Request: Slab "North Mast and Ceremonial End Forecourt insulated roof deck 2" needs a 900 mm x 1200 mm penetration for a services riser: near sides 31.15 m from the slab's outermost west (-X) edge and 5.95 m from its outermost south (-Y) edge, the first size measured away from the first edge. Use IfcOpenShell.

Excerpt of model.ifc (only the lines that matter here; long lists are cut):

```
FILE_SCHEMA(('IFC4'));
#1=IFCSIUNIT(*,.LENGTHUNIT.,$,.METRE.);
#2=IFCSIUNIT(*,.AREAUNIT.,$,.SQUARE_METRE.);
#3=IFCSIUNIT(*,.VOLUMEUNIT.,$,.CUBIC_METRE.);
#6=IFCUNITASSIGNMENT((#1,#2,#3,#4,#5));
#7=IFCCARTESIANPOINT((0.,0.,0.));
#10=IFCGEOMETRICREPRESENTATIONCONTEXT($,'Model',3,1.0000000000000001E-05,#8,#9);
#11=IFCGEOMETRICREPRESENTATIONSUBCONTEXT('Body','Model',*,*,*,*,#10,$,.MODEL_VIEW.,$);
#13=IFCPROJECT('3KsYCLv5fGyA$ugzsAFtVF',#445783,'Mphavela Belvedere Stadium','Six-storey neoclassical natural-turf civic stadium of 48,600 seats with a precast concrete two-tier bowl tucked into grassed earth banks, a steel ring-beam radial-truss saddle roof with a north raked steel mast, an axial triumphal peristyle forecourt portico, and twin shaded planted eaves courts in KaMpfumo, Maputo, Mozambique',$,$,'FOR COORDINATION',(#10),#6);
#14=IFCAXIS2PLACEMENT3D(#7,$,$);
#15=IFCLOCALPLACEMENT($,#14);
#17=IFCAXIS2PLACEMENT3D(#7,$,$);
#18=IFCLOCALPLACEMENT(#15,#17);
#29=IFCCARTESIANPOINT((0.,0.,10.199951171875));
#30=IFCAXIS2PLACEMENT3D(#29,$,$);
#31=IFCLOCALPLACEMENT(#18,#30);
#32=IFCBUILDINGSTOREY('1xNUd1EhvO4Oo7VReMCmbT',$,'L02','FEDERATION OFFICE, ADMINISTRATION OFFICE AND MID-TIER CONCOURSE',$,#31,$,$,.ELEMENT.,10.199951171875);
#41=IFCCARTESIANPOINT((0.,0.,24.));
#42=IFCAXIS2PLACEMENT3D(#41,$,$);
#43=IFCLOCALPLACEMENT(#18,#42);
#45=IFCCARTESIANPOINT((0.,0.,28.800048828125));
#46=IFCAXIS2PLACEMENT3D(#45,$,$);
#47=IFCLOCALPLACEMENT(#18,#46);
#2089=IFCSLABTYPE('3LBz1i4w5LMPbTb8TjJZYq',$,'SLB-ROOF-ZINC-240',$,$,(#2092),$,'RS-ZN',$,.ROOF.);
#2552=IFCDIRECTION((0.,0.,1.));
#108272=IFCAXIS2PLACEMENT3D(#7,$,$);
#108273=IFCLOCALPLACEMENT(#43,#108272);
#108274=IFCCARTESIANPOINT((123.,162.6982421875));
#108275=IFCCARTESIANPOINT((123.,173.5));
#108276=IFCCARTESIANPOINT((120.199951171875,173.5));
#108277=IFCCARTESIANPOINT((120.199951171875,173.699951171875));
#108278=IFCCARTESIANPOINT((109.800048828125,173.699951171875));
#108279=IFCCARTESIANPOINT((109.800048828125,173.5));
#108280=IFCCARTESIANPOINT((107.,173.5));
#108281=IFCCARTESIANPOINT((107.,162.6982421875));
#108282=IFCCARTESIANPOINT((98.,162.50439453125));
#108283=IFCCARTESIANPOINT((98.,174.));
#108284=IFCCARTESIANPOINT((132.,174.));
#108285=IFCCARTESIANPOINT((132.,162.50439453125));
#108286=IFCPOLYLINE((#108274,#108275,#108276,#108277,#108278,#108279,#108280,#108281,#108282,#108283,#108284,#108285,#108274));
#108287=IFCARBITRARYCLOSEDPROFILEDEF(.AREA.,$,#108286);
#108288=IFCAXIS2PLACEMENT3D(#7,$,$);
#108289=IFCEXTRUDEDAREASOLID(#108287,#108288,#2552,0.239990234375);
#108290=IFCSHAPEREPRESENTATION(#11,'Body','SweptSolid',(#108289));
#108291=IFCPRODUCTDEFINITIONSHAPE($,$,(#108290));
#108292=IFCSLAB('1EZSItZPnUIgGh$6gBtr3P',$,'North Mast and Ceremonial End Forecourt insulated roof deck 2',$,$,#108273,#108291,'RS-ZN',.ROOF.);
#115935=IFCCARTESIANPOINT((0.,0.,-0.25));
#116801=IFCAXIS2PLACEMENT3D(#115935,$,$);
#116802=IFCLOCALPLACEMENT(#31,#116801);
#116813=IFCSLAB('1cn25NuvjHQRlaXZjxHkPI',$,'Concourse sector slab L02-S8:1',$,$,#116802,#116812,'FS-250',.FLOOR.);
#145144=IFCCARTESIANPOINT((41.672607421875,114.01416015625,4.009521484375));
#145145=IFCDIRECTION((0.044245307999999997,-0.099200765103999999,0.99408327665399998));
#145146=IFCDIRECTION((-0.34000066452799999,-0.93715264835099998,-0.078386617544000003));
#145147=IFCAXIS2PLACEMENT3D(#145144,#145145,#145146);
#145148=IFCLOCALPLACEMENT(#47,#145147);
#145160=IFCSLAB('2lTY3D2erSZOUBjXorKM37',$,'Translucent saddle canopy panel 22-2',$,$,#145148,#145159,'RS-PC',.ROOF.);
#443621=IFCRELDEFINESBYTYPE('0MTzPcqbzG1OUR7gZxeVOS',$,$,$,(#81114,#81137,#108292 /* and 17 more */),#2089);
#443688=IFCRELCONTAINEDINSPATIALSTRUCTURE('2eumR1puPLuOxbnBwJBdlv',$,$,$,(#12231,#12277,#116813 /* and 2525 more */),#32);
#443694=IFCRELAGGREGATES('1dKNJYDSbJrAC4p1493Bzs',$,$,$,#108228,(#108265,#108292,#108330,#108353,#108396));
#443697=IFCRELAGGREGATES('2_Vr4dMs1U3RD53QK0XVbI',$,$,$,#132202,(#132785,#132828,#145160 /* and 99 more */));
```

```python
import numpy as np
import ifcopenshell
import ifcopenshell.api.feature
import ifcopenshell.api.geometry
import ifcopenshell.api.root
import ifcopenshell.geom
import ifcopenshell.util.placement
import ifcopenshell.util.representation
import ifcopenshell.util.shape
import ifcopenshell.util.unit

model = ifcopenshell.open("model.ifc")
unit_scale = ifcopenshell.util.unit.calculate_unit_scale(model)
settings = ifcopenshell.geom.settings()


def volume(element):
    """Net volume in cubic metres, openings subtracted."""
    shape = ifcopenshell.geom.create_shape(settings, element)
    return ifcopenshell.util.shape.get_volume(shape.geometry)


slab = model.by_guid("1EZSItZPnUIgGh$6gBtr3P")
before = volume(slab)

# Extent in the slab's own axes, in metres. The edges named are its -X and -Y sides.
slab_shape = ifcopenshell.geom.create_shape(settings, slab)
vertices = ifcopenshell.util.shape.get_vertices(slab_shape.geometry)
x_min, y_min, bottom = vertices.min(axis=0)
top = vertices[:, 2].max()

opening = ifcopenshell.api.root.create_entity(model, ifc_class="IfcOpeningElement", name="Services riser opening", predefined_type="OPENING")
context = ifcopenshell.util.representation.get_context(model, "Model", "Body", "MODEL_VIEW")
width, depth = 0.9, 1.2
outline = [(0.0, 0.0), (width, 0.0), (width, depth), (0.0, depth), (0.0, 0.0)]
# Overshoot both faces by 50 mm so the cut is clean.
shape = ifcopenshell.api.geometry.add_slab_representation(
    model, context=context, depth=top - bottom + 0.1, polyline=outline
)
ifcopenshell.api.geometry.assign_representation(model, product=opening, representation=shape)

matrix = ifcopenshell.util.placement.get_local_placement(slab.ObjectPlacement)
matrix[:, 3] = matrix @ np.append(np.array([x_min + 31.15, y_min + 5.95, bottom - 0.05]) / unit_scale, 1.0)
ifcopenshell.api.geometry.edit_object_placement(model, product=opening, matrix=matrix, is_si=False)
ifcopenshell.api.feature.add_feature(model, feature=opening, element=slab)

after = volume(slab)

print(f"slab volume {before:.3f} -> {after:.3f} m3")

model.write("model_updated.ifc")
```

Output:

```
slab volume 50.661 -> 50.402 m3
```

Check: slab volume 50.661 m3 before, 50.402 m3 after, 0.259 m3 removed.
